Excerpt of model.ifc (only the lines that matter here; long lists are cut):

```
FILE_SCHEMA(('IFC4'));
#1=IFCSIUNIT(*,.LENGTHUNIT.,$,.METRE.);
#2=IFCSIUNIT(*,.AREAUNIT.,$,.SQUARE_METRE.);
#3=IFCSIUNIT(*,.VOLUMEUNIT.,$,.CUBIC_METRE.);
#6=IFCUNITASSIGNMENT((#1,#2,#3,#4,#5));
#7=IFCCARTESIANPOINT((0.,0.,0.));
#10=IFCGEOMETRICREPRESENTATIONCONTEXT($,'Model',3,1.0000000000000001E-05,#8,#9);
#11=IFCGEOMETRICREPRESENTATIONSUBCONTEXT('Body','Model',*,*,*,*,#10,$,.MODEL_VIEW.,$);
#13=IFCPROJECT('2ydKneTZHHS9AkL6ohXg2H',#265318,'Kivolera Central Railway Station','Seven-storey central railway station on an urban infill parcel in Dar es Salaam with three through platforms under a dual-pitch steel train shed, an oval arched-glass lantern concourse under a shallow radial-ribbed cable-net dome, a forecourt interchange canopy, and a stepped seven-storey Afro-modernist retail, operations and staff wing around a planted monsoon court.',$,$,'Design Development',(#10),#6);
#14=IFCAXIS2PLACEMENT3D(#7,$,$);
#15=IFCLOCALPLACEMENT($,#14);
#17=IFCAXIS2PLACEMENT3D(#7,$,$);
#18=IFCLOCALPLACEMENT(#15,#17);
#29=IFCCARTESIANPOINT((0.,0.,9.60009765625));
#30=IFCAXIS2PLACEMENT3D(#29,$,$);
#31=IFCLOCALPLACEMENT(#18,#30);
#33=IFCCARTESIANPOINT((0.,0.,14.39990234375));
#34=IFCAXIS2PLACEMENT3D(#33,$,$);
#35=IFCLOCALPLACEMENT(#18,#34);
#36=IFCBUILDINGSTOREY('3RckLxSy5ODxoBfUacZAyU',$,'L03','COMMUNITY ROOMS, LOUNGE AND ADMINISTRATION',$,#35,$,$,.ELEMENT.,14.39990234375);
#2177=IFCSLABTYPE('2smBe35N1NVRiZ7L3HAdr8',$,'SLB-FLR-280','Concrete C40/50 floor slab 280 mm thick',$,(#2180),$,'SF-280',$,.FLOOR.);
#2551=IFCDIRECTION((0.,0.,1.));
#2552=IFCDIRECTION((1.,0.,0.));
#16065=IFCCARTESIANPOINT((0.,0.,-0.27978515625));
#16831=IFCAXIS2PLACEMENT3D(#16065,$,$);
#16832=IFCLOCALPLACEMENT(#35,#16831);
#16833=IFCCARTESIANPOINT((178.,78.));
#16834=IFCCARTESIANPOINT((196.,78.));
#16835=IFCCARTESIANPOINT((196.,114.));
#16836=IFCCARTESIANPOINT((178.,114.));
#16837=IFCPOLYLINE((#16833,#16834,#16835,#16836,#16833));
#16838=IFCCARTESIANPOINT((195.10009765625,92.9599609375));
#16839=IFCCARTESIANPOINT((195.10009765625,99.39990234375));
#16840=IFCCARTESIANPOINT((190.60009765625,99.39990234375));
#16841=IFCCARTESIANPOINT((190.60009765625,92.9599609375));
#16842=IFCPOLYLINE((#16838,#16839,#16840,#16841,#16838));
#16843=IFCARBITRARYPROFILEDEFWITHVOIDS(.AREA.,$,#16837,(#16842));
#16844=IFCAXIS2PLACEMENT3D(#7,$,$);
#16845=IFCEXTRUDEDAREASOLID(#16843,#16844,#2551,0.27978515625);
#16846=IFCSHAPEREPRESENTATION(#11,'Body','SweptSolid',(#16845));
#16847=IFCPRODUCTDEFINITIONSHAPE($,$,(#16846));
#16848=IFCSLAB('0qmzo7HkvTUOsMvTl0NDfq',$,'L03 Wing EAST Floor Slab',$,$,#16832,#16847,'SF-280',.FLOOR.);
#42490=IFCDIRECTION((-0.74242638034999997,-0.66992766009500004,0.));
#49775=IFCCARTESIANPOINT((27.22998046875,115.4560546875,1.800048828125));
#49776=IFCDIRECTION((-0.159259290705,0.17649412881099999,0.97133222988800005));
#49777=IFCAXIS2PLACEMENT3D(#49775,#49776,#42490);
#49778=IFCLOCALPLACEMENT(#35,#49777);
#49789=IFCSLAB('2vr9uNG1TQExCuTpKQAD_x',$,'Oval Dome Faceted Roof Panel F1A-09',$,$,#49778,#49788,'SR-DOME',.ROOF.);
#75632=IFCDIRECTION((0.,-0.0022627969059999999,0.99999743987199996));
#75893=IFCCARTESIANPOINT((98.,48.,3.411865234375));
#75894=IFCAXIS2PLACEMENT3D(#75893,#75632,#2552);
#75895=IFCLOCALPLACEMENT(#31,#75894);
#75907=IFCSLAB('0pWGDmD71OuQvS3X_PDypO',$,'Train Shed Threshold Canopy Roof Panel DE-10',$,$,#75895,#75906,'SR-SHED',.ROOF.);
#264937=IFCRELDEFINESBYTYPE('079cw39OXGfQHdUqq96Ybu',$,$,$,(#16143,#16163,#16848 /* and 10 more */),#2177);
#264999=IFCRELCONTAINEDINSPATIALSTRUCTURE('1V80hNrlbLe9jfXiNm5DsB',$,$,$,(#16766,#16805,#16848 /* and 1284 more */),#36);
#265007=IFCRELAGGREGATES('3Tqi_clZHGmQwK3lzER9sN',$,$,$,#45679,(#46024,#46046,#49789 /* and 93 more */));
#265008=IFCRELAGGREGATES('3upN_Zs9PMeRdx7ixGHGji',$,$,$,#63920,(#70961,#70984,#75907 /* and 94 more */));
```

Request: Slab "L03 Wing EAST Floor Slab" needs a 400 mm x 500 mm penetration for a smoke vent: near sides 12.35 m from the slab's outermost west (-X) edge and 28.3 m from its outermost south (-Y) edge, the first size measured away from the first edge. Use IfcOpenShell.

```python
import numpy as np
import ifcopenshell
import ifcopenshell.api.feature
import ifcopenshell.api.geometry
import ifcopenshell.api.root
import ifcopenshell.geom
import ifcopenshell.util.placement
import ifcopenshell.util.representation
import ifcopenshell.util.shape
import ifcopenshell.util.unit

model = ifcopenshell.open("model.ifc")
unit_scale = ifcopenshell.util.unit.calculate_unit_scale(model)
settings = ifcopenshell.geom.settings()


def volume(element):
    """Net volume in cubic metres, openings subtracted."""
    shape = ifcopenshell.geom.create_shape(settings, element)
    return ifcopenshell.util.shape.get_volume(shape.geometry)


slab = model.by_guid("0qmzo7HkvTUOsMvTl0NDfq")
before = volume(slab)

# Extent in the slab's own axes, in metres. The edges named are its -X and -Y sides.
slab_shape = ifcopenshell.geom.create_shape(settings, slab)
vertices = ifcopenshell.util.shape.get_vertices(slab_shape.geometry)
x_min, y_min, bottom = vertices.min(axis=0)
top = vertices[:, 2].max()

opening = ifcopenshell.api.root.create_entity(model, ifc_class="IfcOpeningElement", name="Smoke vent opening", predefined_type="OPENING")
context = ifcopenshell.util.representation.get_context(model, "Model", "Body", "MODEL_VIEW")
width, depth = 0.4, 0.5
outline = [(0.0, 0.0), (width, 0.0), (width, depth), (0.0, depth), (0.0, 0.0)]
# Overshoot both faces by 50 mm so the cut is clean.
shape = ifcopenshell.api.geometry.add_slab_representation(
    model, context=context, depth=top - bottom + 0.1, polyline=outline
)
ifcopenshell.api.geometry.assign_representation(model, product=opening, representation=shape)

matrix = ifcopenshell.util.placement.get_local_placement(slab.ObjectPlacement)
matrix[:, 3] = matrix @ np.append(np.array([x_min + 12.35, y_min + 28.3, bottom - 0.05]) / unit_scale, 1.0)
ifcopenshell.api.geometry.edit_object_placement(model, product=opening, matrix=matrix, is_si=False)
ifcopenshell.api.feature.add_feature(model, feature=opening, element=slab)

after = volume(slab)

print(f"slab volume {before:.3f} -> {after:.3f} m3")

model.write("model_rev.ifc")
```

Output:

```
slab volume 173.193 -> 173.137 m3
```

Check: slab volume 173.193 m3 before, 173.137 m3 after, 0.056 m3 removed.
